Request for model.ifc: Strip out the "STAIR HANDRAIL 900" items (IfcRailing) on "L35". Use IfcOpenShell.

First a look at what the model holds.

```python
import ifcopenshell
import ifcopenshell.util.element

model = ifcopenshell.open("model.ifc")
print(model.schema)
storey = next(s for s in model.by_type("IfcBuildingStorey") if s.Name == "L35")
railings = [e for e in ifcopenshell.util.element.get_decomposition(storey) if e.is_a("IfcRailing")]
seen = {}
for e in railings:
    element_type = ifcopenshell.util.element.get_type(e)
    name = element_type.Name if element_type not in (None, e) else None
    seen[name] = seen.get(name, 0) + 1
for name, count in sorted(seen.items(), key=str):
    print(count, "x", name)
```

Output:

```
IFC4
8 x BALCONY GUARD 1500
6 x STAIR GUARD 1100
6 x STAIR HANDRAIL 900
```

```python
import ifcopenshell
import ifcopenshell.api.root
import ifcopenshell.util.element

model = ifcopenshell.open("model.ifc")

storey = next(s for s in model.by_type("IfcBuildingStorey") if s.Name == "L35")
railings = [e for e in ifcopenshell.util.element.get_decomposition(storey) if e.is_a("IfcRailing")]
targets = [e for e in railings if (t := ifcopenshell.util.element.get_type(e)) not in (None, e) and t.Name == "STAIR HANDRAIL 900"]

for e in targets:
    ifcopenshell.api.root.remove_product(model, product=e)
print(len(targets), "removed")

model.write("model_rev.ifc")
```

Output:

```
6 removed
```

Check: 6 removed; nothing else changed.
